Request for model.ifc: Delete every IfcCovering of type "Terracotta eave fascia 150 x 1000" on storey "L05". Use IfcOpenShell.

First a look at what the model holds.

```python
import ifcopenshell
import ifcopenshell.util.element

model = ifcopenshell.open("model.ifc")
print(model.schema)
storey = next(s for s in model.by_type("IfcBuildingStorey") if s.Name == "L05")
coverings = [e for e in ifcopenshell.util.element.get_decomposition(storey) if e.is_a("IfcCovering")]
seen = {}
for e in coverings:
    element_type = ifcopenshell.util.element.get_type(e)
    name = element_type.Name if element_type not in (None, e) else None
    seen[name] = seen.get(name, 0) + 1
for name, count in sorted(seen.items(), key=str):
    print(count, "x", name)
```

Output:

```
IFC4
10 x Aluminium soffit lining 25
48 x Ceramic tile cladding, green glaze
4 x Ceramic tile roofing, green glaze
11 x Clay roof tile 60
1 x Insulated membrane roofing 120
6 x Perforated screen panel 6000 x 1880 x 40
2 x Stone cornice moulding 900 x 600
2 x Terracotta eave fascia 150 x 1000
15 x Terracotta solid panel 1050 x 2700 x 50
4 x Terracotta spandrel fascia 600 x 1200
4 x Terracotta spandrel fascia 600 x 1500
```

```python
import ifcopenshell
import ifcopenshell.api.root
import ifcopenshell.util.element

model = ifcopenshell.open("model.ifc")

storey = next(s for s in model.by_type("IfcBuildingStorey") if s.Name == "L05")
coverings = [e for e in ifcopenshell.util.element.get_decomposition(storey) if e.is_a("IfcCovering")]
targets = [e for e in coverings if (t := ifcopenshell.util.element.get_type(e)) not in (None, e) and t.Name == "Terracotta eave fascia 150 x 1000"]

for e in targets:
    ifcopenshell.api.root.remove_product(model, product=e)
print(len(targets), "removed")

model.write("model-out.ifc")
```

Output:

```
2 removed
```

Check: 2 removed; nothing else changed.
